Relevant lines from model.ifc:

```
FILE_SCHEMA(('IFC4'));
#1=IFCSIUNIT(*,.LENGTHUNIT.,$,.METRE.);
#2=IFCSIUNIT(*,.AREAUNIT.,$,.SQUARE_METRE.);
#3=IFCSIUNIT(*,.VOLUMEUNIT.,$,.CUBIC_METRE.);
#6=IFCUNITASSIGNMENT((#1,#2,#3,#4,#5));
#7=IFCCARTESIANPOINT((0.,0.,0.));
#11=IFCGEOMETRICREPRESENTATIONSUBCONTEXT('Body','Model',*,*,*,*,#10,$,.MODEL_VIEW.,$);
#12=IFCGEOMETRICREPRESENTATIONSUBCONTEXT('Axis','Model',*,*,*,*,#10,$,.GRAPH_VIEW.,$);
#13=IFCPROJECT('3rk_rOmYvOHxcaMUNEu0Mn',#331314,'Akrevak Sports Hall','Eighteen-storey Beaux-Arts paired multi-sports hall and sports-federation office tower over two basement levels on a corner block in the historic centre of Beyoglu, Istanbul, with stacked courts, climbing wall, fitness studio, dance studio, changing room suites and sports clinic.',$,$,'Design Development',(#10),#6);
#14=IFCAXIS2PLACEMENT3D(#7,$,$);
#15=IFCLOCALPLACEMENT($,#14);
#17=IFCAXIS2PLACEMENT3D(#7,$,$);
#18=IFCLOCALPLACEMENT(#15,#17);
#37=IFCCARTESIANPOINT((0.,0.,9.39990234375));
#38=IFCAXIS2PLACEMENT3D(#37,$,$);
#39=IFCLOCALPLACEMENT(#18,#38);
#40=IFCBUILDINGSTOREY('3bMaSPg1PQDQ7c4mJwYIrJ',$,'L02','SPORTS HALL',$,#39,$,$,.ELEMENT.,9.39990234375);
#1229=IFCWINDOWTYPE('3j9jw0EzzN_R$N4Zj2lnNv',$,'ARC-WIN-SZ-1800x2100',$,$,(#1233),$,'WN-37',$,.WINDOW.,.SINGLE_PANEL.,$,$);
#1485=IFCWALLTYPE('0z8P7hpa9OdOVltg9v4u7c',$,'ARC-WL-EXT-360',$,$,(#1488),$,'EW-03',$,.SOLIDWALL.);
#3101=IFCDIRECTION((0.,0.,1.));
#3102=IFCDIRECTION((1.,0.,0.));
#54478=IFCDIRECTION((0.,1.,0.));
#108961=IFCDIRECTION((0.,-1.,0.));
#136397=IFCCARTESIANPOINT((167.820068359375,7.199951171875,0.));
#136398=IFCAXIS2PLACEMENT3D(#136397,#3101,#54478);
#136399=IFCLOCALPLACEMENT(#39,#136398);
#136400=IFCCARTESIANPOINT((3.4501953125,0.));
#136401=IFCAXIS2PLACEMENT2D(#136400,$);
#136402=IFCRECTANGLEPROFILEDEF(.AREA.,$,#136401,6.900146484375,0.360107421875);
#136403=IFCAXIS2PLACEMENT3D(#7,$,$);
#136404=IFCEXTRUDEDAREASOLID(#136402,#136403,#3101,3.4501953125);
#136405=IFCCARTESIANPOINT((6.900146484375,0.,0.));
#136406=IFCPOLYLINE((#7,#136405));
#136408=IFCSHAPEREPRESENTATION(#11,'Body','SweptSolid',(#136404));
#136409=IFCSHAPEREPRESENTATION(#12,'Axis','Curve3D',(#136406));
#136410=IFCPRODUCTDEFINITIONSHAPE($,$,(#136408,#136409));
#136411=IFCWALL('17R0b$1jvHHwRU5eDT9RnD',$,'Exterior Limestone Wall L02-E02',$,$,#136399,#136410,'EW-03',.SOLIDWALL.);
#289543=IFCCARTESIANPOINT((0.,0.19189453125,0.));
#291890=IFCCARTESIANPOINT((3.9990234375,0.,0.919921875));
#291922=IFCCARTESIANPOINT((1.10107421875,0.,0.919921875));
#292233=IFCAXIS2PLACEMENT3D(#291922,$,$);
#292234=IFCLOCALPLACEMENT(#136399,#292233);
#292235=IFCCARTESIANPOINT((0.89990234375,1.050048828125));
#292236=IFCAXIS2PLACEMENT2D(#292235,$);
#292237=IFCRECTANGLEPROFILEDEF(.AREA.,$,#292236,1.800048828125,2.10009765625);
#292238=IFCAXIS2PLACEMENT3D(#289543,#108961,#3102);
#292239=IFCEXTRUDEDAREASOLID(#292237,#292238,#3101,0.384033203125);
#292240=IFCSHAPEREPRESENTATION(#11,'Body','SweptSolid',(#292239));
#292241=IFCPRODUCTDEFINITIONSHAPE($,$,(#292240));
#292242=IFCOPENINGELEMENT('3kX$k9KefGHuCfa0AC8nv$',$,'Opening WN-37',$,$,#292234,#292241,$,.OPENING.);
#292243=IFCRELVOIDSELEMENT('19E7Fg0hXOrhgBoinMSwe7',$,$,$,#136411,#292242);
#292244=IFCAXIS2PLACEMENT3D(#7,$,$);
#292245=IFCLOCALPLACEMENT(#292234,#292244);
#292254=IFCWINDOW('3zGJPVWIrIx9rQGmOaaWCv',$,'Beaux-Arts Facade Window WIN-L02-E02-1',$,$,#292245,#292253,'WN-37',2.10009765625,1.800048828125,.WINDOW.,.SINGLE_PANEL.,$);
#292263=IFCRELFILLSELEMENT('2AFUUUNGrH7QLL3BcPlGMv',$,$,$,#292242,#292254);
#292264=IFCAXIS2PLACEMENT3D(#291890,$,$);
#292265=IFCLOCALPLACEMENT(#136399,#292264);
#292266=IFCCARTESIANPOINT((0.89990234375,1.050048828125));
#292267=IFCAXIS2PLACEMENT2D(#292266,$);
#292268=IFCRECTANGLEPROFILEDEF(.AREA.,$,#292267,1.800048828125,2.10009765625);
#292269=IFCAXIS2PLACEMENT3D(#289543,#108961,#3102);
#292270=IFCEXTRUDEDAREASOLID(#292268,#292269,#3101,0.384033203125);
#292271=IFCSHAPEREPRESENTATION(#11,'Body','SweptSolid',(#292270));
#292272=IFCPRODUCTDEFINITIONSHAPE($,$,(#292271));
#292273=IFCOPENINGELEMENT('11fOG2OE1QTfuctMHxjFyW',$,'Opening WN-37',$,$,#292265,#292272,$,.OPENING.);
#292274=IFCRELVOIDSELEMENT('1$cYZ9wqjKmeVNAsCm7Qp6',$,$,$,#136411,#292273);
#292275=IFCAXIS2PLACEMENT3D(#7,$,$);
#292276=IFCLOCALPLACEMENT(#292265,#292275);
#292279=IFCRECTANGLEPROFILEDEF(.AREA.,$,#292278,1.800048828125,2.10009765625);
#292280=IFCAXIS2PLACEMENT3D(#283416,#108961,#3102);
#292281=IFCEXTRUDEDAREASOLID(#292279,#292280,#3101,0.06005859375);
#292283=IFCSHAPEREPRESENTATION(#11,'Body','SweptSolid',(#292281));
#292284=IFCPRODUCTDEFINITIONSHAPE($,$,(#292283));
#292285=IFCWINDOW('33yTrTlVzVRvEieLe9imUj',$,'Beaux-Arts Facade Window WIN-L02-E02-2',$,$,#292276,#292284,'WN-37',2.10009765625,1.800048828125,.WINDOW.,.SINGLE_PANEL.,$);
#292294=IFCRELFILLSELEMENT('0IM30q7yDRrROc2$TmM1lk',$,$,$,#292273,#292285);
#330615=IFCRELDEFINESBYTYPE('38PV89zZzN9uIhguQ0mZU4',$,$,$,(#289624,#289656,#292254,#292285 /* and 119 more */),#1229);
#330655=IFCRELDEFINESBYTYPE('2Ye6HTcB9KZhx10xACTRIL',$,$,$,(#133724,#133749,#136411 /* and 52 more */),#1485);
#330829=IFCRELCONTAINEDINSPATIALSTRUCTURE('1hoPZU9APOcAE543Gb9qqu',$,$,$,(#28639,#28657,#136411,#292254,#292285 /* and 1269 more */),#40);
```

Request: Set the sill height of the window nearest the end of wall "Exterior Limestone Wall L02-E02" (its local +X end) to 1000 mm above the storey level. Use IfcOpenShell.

```python
import numpy as np
import ifcopenshell
import ifcopenshell.api.geometry
import ifcopenshell.geom
import ifcopenshell.util.element
import ifcopenshell.util.placement
import ifcopenshell.util.shape
import ifcopenshell.util.unit

model = ifcopenshell.open("model.ifc")
unit_scale = ifcopenshell.util.unit.calculate_unit_scale(model)

window = model.by_guid("33yTrTlVzVRvEieLe9imUj")
opening = window.FillsVoids[0].RelatingOpeningElement
storey = ifcopenshell.util.element.get_container(window, ifc_class="IfcBuildingStorey")
level = ifcopenshell.util.placement.get_local_placement(storey.ObjectPlacement)[2, 3]

# The opening's origin need not be at the sill, so measure its lowest point.
shape = ifcopenshell.geom.create_shape(ifcopenshell.geom.settings(), opening)
bottom = ifcopenshell.util.shape.get_shape_bottom_elevation(shape, shape.geometry) / unit_scale
dz = level + 1 / unit_scale - bottom

shift = np.array([0.0, 0.0, dz])
# The window is placed relative to its opening, so it follows when the opening moves.
matrix = ifcopenshell.util.placement.get_local_placement(opening.ObjectPlacement)
matrix[:3, 3] += shift
ifcopenshell.api.geometry.edit_object_placement(
    model, product=opening, matrix=matrix, is_si=False, should_transform_children=True
)

print(f"moved by {dz * unit_scale:+.3f} m")

model.write("model-out.ifc")
```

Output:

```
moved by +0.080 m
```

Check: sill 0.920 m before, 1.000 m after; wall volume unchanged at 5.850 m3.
